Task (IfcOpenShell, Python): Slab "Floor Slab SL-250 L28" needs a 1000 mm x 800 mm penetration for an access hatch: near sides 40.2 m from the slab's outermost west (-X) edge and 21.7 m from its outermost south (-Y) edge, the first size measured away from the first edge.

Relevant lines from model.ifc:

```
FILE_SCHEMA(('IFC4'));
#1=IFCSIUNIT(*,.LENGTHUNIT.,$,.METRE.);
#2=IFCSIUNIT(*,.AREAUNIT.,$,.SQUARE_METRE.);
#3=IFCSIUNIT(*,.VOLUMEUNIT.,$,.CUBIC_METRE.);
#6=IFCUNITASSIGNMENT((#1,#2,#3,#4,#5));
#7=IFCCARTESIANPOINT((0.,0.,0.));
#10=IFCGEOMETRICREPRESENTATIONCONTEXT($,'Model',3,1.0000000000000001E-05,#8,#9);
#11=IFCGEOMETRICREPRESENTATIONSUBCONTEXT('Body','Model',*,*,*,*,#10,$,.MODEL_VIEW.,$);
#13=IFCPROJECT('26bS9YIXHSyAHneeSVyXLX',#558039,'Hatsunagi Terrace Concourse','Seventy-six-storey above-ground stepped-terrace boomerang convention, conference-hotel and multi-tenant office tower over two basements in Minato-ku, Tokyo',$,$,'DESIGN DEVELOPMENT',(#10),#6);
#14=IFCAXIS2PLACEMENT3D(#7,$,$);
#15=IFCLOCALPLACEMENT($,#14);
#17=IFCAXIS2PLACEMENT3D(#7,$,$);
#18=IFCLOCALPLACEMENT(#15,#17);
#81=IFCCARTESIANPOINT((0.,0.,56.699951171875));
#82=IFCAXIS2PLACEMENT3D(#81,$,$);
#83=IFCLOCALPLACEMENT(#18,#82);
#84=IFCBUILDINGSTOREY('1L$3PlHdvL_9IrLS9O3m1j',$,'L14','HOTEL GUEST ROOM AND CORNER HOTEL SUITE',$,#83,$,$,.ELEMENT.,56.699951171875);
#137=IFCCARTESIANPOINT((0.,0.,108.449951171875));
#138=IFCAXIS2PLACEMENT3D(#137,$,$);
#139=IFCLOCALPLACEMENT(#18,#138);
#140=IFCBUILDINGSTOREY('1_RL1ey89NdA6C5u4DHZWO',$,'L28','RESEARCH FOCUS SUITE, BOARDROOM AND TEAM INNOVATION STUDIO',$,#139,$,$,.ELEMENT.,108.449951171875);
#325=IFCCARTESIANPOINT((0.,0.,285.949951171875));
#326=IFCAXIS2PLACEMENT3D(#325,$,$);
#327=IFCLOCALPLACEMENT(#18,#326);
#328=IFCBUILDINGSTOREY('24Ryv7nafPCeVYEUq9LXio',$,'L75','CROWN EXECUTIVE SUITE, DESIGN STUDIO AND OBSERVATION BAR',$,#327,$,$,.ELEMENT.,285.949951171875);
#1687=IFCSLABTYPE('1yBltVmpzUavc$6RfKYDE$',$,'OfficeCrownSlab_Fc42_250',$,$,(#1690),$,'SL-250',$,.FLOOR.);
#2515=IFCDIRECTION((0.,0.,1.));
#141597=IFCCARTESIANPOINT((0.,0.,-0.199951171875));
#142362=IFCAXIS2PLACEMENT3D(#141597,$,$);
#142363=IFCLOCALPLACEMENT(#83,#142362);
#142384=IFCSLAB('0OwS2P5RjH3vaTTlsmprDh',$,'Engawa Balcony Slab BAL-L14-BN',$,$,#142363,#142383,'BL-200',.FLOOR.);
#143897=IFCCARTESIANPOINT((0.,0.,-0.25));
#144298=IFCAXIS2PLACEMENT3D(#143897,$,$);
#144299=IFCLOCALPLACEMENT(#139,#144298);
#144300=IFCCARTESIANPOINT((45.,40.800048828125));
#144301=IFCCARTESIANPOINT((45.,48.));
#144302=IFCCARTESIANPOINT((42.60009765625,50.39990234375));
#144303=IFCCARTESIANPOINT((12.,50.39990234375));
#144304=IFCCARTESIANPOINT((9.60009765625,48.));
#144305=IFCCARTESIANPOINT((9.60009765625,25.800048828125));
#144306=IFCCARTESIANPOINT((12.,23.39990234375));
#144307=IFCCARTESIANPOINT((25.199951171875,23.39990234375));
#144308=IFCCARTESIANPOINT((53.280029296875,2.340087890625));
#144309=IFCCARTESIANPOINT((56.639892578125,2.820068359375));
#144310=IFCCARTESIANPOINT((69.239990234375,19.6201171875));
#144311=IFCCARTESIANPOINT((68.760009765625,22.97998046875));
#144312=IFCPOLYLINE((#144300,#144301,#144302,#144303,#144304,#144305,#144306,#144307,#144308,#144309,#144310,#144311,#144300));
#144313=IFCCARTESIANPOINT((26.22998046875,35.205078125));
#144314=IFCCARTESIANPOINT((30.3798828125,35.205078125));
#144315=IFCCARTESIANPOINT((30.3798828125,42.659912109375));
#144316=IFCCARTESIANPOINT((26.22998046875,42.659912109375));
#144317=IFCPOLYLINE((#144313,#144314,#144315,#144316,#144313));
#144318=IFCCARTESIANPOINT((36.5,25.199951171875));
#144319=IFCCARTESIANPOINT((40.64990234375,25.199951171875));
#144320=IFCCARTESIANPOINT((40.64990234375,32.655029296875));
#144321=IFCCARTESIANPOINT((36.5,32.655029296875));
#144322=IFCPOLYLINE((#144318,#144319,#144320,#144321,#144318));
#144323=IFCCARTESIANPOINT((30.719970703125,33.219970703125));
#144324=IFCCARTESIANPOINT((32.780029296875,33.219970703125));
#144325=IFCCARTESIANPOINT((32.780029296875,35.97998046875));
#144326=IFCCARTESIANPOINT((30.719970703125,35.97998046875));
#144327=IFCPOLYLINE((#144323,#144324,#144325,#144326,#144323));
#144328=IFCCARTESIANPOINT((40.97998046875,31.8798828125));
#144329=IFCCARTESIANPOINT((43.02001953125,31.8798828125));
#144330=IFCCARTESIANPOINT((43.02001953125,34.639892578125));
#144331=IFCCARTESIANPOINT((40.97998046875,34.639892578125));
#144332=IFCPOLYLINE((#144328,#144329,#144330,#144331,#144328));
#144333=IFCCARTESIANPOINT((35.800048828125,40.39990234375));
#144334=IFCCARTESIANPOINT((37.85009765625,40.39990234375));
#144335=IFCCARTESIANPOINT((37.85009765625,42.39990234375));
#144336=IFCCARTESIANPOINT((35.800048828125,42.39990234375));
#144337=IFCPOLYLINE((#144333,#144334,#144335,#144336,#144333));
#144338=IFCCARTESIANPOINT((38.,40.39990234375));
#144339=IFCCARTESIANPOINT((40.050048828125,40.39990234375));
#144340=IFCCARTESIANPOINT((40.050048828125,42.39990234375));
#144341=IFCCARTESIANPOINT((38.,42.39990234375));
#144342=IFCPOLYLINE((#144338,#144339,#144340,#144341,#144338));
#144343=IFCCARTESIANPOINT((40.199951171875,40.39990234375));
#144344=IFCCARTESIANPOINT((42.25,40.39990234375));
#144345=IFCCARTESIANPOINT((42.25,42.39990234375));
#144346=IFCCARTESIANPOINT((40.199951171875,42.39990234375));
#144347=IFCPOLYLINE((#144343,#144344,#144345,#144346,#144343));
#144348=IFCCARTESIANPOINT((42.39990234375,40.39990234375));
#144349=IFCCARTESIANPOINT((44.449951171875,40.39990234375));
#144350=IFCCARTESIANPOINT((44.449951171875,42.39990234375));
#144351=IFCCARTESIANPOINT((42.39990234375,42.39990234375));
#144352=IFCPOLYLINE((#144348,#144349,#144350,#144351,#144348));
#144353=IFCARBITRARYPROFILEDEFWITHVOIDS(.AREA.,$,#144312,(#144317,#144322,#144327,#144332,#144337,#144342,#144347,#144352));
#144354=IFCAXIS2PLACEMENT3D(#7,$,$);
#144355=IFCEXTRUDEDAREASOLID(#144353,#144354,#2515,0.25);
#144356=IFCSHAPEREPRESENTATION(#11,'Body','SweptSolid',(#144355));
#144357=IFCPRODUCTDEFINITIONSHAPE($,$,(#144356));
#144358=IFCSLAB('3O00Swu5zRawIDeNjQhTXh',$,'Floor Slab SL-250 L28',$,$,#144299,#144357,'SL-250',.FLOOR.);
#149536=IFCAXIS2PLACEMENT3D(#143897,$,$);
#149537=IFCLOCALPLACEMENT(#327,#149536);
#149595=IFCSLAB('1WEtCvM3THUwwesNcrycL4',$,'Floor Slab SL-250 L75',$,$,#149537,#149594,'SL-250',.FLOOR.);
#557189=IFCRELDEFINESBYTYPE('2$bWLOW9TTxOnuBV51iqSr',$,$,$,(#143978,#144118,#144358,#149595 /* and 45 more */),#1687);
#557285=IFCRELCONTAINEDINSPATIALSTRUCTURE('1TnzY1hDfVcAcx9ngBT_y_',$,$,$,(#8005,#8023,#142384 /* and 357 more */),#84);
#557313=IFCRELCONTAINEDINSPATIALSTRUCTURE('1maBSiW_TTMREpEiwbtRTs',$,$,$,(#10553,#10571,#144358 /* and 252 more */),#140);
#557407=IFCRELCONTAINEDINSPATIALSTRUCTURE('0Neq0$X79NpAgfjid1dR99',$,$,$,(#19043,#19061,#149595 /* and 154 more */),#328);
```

```python
import numpy as np
import ifcopenshell
import ifcopenshell.api.feature
import ifcopenshell.api.geometry
import ifcopenshell.api.root
import ifcopenshell.geom
import ifcopenshell.util.placement
import ifcopenshell.util.representation
import ifcopenshell.util.shape
import ifcopenshell.util.unit

model = ifcopenshell.open("model.ifc")
unit_scale = ifcopenshell.util.unit.calculate_unit_scale(model)
settings = ifcopenshell.geom.settings()


def volume(element):
    """Net volume in cubic metres, openings subtracted."""
    shape = ifcopenshell.geom.create_shape(settings, element)
    return ifcopenshell.util.shape.get_volume(shape.geometry)


slab = model.by_guid("3O00Swu5zRawIDeNjQhTXh")
before = volume(slab)

# Extent in the slab's own axes, in metres. The edges named are its -X and -Y sides.
slab_shape = ifcopenshell.geom.create_shape(settings, slab)
vertices = ifcopenshell.util.shape.get_vertices(slab_shape.geometry)
x_min, y_min, bottom = vertices.min(axis=0)
top = vertices[:, 2].max()

opening = ifcopenshell.api.root.create_entity(model, ifc_class="IfcOpeningElement", name="Access hatch opening", predefined_type="OPENING")
context = ifcopenshell.util.representation.get_context(model, "Model", "Body", "MODEL_VIEW")
width, depth = 1, 0.8
outline = [(0.0, 0.0), (width, 0.0), (width, depth), (0.0, depth), (0.0, 0.0)]
# Overshoot both faces by 50 mm so the cut is clean.
shape = ifcopenshell.api.geometry.add_slab_representation(
    model, context=context, depth=top - bottom + 0.1, polyline=outline
)
ifcopenshell.api.geometry.assign_representation(model, product=opening, representation=shape)

matrix = ifcopenshell.util.placement.get_local_placement(slab.ObjectPlacement)
matrix[:, 3] = matrix @ np.append(np.array([x_min + 40.2, y_min + 21.7, bottom - 0.05]) / unit_scale, 1.0)
ifcopenshell.api.geometry.edit_object_placement(model, product=opening, matrix=matrix, is_si=False)
ifcopenshell.api.feature.add_feature(model, feature=opening, element=slab)

after = volume(slab)

print(f"slab volume {before:.3f} -> {after:.3f} m3")

model.write("model_updated.ifc")
```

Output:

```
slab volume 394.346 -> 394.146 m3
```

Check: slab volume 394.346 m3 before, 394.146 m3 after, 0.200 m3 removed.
